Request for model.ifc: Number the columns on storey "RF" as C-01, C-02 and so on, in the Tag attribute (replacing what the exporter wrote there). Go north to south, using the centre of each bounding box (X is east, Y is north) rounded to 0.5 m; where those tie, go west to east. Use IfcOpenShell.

First a look at what the model holds.

```python
import ifcopenshell
import ifcopenshell.util.element
import ifcopenshell.util.placement

model = ifcopenshell.open("model.ifc")
print(model.schema)
storey = next(s for s in model.by_type("IfcBuildingStorey") if s.Name == "RF")
columns = [e for e in ifcopenshell.util.element.get_decomposition(storey) if e.is_a("IfcColumn")]
for e in sorted(columns, key=lambda e: e.id()):
    origin = ifcopenshell.util.placement.get_local_placement(e.ObjectPlacement)[:3, 3]
    print(e.id(), e.Tag, e.Name, origin.round(2) + 0.0, sep=" | ")
```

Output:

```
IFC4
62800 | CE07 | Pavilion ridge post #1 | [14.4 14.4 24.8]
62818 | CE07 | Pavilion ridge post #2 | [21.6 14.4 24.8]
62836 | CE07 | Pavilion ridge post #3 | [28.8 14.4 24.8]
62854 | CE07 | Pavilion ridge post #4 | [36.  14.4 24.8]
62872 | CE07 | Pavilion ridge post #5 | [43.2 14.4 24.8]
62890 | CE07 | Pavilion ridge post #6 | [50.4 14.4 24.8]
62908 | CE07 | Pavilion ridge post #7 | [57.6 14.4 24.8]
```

```python
import ifcopenshell
import ifcopenshell.geom
import ifcopenshell.util.element
import ifcopenshell.util.shape

model = ifcopenshell.open("model.ifc")
settings = ifcopenshell.geom.settings()
settings.set("use-world-coords", True)


def centre(element):
    shape = ifcopenshell.geom.create_shape(settings, element)
    return ifcopenshell.util.shape.get_bbox_centroid(shape.geometry)


storey = next(s for s in model.by_type("IfcBuildingStorey") if s.Name == "RF")
columns = [e for e in ifcopenshell.util.element.get_decomposition(storey) if e.is_a("IfcColumn")]

# Insertion points can sit at a corner or the storey origin, so sort by the geometry (in metres).
centres = {e: centre(e) for e in columns}
columns.sort(key=lambda e: (-round(centres[e][1] / 0.5), centres[e][0]))

for i, e in enumerate(columns, start=1):
    number = f"C-{i:02d}"
    e.Tag = number
    print(e.id(), number)

model.write("model_updated.ifc")
```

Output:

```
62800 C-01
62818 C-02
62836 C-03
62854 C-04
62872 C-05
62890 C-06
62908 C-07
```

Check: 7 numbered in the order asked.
